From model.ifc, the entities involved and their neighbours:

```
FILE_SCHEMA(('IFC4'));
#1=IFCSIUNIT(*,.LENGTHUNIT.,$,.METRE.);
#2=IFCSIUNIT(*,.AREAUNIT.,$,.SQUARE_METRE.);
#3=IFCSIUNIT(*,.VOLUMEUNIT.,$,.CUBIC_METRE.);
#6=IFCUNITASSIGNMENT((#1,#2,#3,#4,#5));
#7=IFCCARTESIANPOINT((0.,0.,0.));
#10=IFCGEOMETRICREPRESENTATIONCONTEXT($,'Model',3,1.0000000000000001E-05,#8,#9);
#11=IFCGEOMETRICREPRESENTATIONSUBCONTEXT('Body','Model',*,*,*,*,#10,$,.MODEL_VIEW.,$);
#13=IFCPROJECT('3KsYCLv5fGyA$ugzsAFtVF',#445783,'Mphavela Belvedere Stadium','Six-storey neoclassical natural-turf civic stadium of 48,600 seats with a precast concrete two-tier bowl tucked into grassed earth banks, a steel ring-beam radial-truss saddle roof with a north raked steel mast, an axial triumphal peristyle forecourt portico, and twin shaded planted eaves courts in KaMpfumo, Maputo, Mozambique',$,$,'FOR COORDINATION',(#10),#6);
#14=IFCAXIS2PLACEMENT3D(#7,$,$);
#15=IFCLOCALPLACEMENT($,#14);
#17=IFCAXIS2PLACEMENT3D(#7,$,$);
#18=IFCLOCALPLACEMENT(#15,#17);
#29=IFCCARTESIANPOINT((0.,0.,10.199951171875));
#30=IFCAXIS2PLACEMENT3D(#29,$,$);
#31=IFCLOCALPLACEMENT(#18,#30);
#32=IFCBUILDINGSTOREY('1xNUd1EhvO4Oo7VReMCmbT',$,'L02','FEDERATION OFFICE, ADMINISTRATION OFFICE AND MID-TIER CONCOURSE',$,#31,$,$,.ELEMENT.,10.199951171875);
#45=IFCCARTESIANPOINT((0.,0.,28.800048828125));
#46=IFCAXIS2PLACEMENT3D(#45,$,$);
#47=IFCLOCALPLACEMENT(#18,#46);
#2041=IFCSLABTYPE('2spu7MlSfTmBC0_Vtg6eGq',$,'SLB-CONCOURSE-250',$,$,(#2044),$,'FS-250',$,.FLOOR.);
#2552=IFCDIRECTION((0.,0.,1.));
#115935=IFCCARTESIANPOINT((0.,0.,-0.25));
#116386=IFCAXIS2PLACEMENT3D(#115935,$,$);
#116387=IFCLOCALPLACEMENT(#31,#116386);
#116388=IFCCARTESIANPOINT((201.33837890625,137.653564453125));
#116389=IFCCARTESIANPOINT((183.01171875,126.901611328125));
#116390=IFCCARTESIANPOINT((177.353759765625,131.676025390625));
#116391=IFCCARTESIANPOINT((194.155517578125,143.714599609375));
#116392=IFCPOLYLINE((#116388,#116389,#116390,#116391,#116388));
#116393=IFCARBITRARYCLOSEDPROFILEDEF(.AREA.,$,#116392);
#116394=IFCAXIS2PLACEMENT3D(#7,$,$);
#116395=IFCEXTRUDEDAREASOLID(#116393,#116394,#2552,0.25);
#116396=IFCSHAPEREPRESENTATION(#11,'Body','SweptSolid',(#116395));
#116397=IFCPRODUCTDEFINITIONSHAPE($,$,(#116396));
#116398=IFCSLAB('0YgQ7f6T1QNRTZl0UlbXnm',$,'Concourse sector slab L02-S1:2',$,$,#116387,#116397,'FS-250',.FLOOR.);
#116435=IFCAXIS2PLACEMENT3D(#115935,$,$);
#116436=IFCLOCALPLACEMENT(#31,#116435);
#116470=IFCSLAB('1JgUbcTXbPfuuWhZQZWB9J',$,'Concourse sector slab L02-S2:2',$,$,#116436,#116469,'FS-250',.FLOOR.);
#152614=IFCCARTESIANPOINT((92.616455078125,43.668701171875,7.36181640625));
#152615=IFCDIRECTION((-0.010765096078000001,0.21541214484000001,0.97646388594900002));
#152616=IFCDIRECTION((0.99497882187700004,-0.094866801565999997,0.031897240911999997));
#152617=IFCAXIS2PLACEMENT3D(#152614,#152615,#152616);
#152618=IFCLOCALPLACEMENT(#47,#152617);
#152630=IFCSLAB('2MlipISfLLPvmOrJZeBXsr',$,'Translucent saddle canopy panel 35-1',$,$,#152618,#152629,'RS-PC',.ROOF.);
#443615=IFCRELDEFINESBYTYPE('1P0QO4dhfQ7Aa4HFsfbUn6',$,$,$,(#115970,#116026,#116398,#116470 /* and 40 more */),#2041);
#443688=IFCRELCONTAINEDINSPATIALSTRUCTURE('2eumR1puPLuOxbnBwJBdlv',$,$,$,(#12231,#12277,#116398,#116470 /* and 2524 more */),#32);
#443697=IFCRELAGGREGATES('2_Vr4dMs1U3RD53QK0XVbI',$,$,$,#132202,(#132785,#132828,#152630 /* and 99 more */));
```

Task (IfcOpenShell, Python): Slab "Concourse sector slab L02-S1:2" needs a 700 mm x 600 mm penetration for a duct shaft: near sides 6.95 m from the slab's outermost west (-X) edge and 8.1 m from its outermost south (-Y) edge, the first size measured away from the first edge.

```python
import numpy as np
import ifcopenshell
import ifcopenshell.api.feature
import ifcopenshell.api.geometry
import ifcopenshell.api.root
import ifcopenshell.geom
import ifcopenshell.util.placement
import ifcopenshell.util.representation
import ifcopenshell.util.shape
import ifcopenshell.util.unit

model = ifcopenshell.open("model.ifc")
unit_scale = ifcopenshell.util.unit.calculate_unit_scale(model)
settings = ifcopenshell.geom.settings()


def volume(element):
    """Net volume in cubic metres, openings subtracted."""
    shape = ifcopenshell.geom.create_shape(settings, element)
    return ifcopenshell.util.shape.get_volume(shape.geometry)


slab = model.by_guid("0YgQ7f6T1QNRTZl0UlbXnm")
before = volume(slab)

# Extent in the slab's own axes, in metres. The edges named are its -X and -Y sides.
slab_shape = ifcopenshell.geom.create_shape(settings, slab)
vertices = ifcopenshell.util.shape.get_vertices(slab_shape.geometry)
x_min, y_min, bottom = vertices.min(axis=0)
top = vertices[:, 2].max()

opening = ifcopenshell.api.root.create_entity(model, ifc_class="IfcOpeningElement", name="Duct shaft opening", predefined_type="OPENING")
context = ifcopenshell.util.representation.get_context(model, "Model", "Body", "MODEL_VIEW")
width, depth = 0.7, 0.6
outline = [(0.0, 0.0), (width, 0.0), (width, depth), (0.0, depth), (0.0, 0.0)]
# Overshoot both faces by 50 mm so the cut is clean.
shape = ifcopenshell.api.geometry.add_slab_representation(
    model, context=context, depth=top - bottom + 0.1, polyline=outline
)
ifcopenshell.api.geometry.assign_representation(model, product=opening, representation=shape)

matrix = ifcopenshell.util.placement.get_local_placement(slab.ObjectPlacement)
matrix[:, 3] = matrix @ np.append(np.array([x_min + 6.95, y_min + 8.1, bottom - 0.05]) / unit_scale, 1.0)
ifcopenshell.api.geometry.edit_object_placement(model, product=opening, matrix=matrix, is_si=False)
ifcopenshell.api.feature.add_feature(model, feature=opening, element=slab)

after = volume(slab)

print(f"slab volume {before:.3f} -> {after:.3f} m3")

model.write("model_updated.ifc")
```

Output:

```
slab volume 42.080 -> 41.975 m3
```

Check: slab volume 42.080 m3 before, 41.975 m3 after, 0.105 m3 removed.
